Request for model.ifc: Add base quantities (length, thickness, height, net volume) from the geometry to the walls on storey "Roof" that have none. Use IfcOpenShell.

First a look at what the model holds.

```python
import ifcopenshell
import ifcopenshell.util.element
import ifcopenshell.util.unit

model = ifcopenshell.open("model.ifc")
print(model.schema)
for unit_type in ("LENGTHUNIT", "AREAUNIT", "VOLUMEUNIT"):
    print(unit_type, ifcopenshell.util.unit.calculate_unit_scale(model, unit_type))
storey = next(s for s in model.by_type("IfcBuildingStorey") if s.Name == "Roof")
walls = [e for e in ifcopenshell.util.element.get_decomposition(storey) if e.is_a("IfcWall")]
for e in sorted(walls, key=lambda e: e.id()):
    print(e.id(), e.is_a(), e.Name, list(ifcopenshell.util.element.get_psets(e, qtos_only=True)), sep=" | ")
```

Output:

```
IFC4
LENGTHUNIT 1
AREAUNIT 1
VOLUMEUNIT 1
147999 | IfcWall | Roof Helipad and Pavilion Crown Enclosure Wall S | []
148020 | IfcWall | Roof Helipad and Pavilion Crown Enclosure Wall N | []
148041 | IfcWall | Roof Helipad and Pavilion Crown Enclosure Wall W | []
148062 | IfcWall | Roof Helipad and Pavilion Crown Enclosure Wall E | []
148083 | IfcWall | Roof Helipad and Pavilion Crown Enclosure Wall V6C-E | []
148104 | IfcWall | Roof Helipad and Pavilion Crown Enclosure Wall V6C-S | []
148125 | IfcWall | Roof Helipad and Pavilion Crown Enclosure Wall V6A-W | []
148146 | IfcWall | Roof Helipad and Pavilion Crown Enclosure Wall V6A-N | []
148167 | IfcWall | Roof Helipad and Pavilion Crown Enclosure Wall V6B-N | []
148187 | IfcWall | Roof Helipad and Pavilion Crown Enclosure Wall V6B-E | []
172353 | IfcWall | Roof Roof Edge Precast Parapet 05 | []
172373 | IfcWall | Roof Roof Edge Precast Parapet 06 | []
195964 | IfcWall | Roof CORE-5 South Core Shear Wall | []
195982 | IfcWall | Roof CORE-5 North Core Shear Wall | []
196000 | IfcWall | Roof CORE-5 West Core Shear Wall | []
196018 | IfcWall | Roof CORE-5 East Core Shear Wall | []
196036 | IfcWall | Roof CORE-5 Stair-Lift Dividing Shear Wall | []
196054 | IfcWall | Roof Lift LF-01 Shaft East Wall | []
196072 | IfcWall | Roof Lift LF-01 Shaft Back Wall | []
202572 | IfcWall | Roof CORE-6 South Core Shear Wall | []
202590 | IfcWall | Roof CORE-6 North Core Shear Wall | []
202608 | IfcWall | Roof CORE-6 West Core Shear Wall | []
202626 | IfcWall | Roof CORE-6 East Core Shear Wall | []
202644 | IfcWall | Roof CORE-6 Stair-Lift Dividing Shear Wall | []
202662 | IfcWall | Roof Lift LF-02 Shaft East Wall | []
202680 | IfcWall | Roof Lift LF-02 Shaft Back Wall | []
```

```python
import ifcopenshell
import ifcopenshell.api.pset
import ifcopenshell.geom
import ifcopenshell.util.element
import ifcopenshell.util.shape
import ifcopenshell.util.unit

model = ifcopenshell.open("model.ifc")
unit_scale = ifcopenshell.util.unit.calculate_unit_scale(model)
volume_scale = ifcopenshell.util.unit.calculate_unit_scale(model, "VOLUMEUNIT")
settings = ifcopenshell.geom.settings()

storey = next(s for s in model.by_type("IfcBuildingStorey") if s.Name == "Roof")
walls = [e for e in ifcopenshell.util.element.get_decomposition(storey) if e.is_a("IfcWall")]

for e in sorted(walls, key=lambda e: e.id()):
    if ifcopenshell.util.element.get_psets(e, qtos_only=True, should_inherit=False):
        continue
    # Geometry comes back in metres, in the element's own axes.
    shape = ifcopenshell.geom.create_shape(settings, e)
    values = {
        "Length": ifcopenshell.util.shape.get_x(shape.geometry) / unit_scale,
        "Width": ifcopenshell.util.shape.get_y(shape.geometry) / unit_scale,
        "Height": ifcopenshell.util.shape.get_z(shape.geometry) / unit_scale,
        "NetVolume": ifcopenshell.util.shape.get_volume(shape.geometry) / volume_scale,
    }
    qto = ifcopenshell.api.pset.add_qto(model, product=e, name="Qto_WallBaseQuantities")
    ifcopenshell.api.pset.edit_qto(model, qto=qto, properties=values)
    print(e.id(), {k: round(v, 3) for k, v in values.items()})

model.write("model-out.ifc")
```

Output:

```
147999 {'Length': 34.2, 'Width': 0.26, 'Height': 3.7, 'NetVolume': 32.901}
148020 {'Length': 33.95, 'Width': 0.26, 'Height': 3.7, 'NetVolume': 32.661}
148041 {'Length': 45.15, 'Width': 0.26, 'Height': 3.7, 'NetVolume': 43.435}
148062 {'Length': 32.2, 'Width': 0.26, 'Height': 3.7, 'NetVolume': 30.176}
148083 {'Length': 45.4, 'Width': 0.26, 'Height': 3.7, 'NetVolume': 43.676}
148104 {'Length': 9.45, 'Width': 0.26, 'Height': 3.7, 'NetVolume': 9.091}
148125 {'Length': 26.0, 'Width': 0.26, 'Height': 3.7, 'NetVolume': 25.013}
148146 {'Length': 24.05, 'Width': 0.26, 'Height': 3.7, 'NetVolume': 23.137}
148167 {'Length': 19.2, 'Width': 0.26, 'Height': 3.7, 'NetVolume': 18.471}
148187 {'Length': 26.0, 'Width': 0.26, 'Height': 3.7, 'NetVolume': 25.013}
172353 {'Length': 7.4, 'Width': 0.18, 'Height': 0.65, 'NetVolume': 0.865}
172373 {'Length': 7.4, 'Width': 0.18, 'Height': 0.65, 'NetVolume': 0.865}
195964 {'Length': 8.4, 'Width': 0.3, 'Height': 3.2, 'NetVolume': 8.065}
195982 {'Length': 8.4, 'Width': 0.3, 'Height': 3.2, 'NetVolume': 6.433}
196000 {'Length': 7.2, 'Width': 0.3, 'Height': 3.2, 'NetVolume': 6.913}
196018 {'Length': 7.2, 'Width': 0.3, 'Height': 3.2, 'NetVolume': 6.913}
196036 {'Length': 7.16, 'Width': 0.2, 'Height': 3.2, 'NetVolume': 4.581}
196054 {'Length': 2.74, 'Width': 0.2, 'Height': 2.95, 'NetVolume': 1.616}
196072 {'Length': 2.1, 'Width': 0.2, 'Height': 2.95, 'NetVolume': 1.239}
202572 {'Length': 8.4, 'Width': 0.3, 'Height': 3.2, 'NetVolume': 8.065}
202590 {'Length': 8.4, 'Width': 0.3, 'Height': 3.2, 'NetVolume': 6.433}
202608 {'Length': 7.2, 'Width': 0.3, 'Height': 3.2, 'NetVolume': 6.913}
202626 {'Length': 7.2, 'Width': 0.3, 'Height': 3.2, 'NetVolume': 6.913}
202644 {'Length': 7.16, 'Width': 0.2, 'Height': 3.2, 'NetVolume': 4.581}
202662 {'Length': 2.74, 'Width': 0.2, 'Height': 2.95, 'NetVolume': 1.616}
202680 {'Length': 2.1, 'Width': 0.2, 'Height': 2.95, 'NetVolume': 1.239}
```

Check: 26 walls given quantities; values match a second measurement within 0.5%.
